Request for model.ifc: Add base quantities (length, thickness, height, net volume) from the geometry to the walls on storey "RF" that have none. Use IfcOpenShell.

First a look at what the model holds.

```python
import ifcopenshell
import ifcopenshell.util.element
import ifcopenshell.util.unit

model = ifcopenshell.open("model.ifc")
print(model.schema)
for unit_type in ("LENGTHUNIT", "AREAUNIT", "VOLUMEUNIT"):
    print(unit_type, ifcopenshell.util.unit.calculate_unit_scale(model, unit_type))
storey = next(s for s in model.by_type("IfcBuildingStorey") if s.Name == "RF")
walls = [e for e in ifcopenshell.util.element.get_decomposition(storey) if e.is_a("IfcWall")]
for e in sorted(walls, key=lambda e: e.id()):
    print(e.id(), e.is_a(), e.Name, list(ifcopenshell.util.element.get_psets(e, qtos_only=True)), sep=" | ")
```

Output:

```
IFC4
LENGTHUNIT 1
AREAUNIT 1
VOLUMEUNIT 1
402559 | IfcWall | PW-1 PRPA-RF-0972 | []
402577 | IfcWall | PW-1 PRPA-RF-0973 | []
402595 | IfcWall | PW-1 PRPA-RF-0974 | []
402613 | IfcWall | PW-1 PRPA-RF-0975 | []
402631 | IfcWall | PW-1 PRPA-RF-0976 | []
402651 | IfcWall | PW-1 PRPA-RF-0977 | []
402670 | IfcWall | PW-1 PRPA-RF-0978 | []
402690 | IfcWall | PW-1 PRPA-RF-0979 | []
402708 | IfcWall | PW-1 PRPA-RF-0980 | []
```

```python
import ifcopenshell
import ifcopenshell.api.pset
import ifcopenshell.geom
import ifcopenshell.util.element
import ifcopenshell.util.shape
import ifcopenshell.util.unit

model = ifcopenshell.open("model.ifc")
unit_scale = ifcopenshell.util.unit.calculate_unit_scale(model)
volume_scale = ifcopenshell.util.unit.calculate_unit_scale(model, "VOLUMEUNIT")
settings = ifcopenshell.geom.settings()

storey = next(s for s in model.by_type("IfcBuildingStorey") if s.Name == "RF")
walls = [e for e in ifcopenshell.util.element.get_decomposition(storey) if e.is_a("IfcWall")]

for e in sorted(walls, key=lambda e: e.id()):
    if ifcopenshell.util.element.get_psets(e, qtos_only=True, should_inherit=False):
        continue
    # Geometry comes back in metres, in the element's own axes.
    shape = ifcopenshell.geom.create_shape(settings, e)
    values = {
        "Length": ifcopenshell.util.shape.get_x(shape.geometry) / unit_scale,
        "Width": ifcopenshell.util.shape.get_y(shape.geometry) / unit_scale,
        "Height": ifcopenshell.util.shape.get_z(shape.geometry) / unit_scale,
        "NetVolume": ifcopenshell.util.shape.get_volume(shape.geometry) / volume_scale,
    }
    qto = ifcopenshell.api.pset.add_qto(model, product=e, name="Qto_WallBaseQuantities")
    ifcopenshell.api.pset.edit_qto(model, qto=qto, properties=values)
    print(e.id(), {k: round(v, 3) for k, v in values.items()})

model.write("model-out.ifc")
```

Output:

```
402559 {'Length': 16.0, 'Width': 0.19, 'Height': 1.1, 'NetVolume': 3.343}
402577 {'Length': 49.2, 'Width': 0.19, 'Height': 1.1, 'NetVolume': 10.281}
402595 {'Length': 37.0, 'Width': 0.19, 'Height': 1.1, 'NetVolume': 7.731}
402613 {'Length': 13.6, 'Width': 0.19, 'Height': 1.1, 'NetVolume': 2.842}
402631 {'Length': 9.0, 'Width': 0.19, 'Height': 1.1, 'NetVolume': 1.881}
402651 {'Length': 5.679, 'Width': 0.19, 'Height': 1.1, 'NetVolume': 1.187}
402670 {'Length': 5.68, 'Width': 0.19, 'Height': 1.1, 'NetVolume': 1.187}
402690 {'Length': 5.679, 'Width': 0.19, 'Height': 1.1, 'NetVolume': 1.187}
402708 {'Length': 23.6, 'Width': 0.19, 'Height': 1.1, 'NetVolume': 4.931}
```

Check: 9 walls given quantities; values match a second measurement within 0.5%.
